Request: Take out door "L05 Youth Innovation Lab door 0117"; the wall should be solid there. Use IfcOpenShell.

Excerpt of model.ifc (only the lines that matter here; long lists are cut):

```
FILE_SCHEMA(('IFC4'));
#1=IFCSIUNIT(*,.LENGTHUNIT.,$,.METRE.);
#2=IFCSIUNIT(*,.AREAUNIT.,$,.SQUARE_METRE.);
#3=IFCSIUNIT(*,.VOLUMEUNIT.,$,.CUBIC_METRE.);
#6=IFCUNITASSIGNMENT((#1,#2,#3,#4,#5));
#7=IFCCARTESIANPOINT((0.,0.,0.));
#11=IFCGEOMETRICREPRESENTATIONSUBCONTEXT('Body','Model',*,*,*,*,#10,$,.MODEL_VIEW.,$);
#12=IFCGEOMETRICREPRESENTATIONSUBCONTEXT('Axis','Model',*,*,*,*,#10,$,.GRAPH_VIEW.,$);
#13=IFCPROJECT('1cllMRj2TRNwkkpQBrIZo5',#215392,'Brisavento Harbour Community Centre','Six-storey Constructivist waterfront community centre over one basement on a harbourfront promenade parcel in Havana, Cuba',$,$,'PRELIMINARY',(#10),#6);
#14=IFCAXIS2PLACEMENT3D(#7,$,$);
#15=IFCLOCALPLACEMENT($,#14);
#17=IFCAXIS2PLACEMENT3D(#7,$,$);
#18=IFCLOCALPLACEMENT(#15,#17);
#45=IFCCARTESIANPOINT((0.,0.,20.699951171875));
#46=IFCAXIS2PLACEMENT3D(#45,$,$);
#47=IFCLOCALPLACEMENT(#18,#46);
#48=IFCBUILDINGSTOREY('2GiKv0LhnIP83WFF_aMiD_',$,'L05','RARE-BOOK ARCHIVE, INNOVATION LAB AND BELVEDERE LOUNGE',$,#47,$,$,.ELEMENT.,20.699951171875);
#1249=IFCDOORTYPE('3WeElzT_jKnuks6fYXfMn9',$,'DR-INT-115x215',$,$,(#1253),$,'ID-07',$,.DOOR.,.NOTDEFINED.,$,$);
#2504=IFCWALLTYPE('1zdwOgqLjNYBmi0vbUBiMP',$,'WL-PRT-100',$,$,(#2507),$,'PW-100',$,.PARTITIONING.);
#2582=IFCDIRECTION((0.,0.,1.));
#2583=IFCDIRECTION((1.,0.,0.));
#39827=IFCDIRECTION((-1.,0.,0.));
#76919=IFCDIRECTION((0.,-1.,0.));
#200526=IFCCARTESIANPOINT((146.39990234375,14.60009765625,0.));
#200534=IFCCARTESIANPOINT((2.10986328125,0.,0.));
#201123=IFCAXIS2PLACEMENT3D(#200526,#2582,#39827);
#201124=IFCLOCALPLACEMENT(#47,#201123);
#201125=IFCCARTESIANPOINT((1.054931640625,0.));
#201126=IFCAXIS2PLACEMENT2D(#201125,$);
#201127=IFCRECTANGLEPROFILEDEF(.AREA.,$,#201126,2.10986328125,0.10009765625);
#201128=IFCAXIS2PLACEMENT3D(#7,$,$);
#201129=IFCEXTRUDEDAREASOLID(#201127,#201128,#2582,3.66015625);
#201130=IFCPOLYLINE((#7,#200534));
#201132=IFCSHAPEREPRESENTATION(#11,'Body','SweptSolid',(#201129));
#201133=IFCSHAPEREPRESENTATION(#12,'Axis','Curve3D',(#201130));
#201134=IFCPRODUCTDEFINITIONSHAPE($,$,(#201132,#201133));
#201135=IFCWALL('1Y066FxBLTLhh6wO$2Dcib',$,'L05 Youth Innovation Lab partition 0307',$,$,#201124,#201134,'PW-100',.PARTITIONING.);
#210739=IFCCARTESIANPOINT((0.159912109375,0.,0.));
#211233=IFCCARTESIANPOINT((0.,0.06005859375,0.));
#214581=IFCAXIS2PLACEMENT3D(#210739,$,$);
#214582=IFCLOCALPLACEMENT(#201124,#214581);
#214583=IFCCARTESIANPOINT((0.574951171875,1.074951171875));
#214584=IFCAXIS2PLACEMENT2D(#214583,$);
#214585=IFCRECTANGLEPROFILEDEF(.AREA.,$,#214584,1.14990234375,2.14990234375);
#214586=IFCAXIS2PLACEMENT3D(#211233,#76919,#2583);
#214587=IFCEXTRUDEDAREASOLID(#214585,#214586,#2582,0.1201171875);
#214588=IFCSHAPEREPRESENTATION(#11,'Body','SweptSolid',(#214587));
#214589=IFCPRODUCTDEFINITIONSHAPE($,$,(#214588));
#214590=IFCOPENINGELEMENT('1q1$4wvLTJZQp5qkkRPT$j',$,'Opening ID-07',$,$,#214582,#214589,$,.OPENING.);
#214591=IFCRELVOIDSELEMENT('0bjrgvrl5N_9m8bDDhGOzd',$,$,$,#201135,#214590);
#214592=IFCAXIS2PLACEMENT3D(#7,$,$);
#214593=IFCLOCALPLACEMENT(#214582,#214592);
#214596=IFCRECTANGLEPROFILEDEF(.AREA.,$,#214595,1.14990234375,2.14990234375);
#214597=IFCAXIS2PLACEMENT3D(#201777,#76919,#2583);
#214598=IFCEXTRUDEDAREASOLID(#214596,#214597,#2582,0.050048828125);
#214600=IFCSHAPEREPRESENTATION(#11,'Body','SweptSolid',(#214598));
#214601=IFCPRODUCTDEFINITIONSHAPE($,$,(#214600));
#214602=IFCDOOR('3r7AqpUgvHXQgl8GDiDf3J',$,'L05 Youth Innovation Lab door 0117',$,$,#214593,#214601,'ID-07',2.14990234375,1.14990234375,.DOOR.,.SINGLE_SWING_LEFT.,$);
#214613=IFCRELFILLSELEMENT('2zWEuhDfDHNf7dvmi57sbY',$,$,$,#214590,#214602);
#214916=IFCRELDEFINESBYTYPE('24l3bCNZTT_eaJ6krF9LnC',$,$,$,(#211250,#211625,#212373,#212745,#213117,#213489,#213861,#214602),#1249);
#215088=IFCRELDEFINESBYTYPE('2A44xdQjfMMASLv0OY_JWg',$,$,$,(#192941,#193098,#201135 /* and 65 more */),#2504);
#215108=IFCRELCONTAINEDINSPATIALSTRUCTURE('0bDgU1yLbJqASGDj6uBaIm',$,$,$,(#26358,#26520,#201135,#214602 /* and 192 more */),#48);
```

```python
import ifcopenshell
import ifcopenshell.api.feature
import ifcopenshell.api.root
import ifcopenshell.geom
import ifcopenshell.util.shape

model = ifcopenshell.open("model.ifc")
settings = ifcopenshell.geom.settings()


def volume(element):
    """Net volume in cubic metres, openings subtracted."""
    shape = ifcopenshell.geom.create_shape(settings, element)
    return ifcopenshell.util.shape.get_volume(shape.geometry)


door = model.by_id(214602)
opening = door.FillsVoids[0].RelatingOpeningElement
wall = opening.VoidsElements[0].RelatingBuildingElement
before = volume(wall)

ifcopenshell.api.root.remove_product(model, product=door)
ifcopenshell.api.feature.remove_feature(model, feature=opening)

after = volume(wall)

print(f"wall volume {before:.3f} -> {after:.3f} m3")

model.write("model_rev.ifc")
```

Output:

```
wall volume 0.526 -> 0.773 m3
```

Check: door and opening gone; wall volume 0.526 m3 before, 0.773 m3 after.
